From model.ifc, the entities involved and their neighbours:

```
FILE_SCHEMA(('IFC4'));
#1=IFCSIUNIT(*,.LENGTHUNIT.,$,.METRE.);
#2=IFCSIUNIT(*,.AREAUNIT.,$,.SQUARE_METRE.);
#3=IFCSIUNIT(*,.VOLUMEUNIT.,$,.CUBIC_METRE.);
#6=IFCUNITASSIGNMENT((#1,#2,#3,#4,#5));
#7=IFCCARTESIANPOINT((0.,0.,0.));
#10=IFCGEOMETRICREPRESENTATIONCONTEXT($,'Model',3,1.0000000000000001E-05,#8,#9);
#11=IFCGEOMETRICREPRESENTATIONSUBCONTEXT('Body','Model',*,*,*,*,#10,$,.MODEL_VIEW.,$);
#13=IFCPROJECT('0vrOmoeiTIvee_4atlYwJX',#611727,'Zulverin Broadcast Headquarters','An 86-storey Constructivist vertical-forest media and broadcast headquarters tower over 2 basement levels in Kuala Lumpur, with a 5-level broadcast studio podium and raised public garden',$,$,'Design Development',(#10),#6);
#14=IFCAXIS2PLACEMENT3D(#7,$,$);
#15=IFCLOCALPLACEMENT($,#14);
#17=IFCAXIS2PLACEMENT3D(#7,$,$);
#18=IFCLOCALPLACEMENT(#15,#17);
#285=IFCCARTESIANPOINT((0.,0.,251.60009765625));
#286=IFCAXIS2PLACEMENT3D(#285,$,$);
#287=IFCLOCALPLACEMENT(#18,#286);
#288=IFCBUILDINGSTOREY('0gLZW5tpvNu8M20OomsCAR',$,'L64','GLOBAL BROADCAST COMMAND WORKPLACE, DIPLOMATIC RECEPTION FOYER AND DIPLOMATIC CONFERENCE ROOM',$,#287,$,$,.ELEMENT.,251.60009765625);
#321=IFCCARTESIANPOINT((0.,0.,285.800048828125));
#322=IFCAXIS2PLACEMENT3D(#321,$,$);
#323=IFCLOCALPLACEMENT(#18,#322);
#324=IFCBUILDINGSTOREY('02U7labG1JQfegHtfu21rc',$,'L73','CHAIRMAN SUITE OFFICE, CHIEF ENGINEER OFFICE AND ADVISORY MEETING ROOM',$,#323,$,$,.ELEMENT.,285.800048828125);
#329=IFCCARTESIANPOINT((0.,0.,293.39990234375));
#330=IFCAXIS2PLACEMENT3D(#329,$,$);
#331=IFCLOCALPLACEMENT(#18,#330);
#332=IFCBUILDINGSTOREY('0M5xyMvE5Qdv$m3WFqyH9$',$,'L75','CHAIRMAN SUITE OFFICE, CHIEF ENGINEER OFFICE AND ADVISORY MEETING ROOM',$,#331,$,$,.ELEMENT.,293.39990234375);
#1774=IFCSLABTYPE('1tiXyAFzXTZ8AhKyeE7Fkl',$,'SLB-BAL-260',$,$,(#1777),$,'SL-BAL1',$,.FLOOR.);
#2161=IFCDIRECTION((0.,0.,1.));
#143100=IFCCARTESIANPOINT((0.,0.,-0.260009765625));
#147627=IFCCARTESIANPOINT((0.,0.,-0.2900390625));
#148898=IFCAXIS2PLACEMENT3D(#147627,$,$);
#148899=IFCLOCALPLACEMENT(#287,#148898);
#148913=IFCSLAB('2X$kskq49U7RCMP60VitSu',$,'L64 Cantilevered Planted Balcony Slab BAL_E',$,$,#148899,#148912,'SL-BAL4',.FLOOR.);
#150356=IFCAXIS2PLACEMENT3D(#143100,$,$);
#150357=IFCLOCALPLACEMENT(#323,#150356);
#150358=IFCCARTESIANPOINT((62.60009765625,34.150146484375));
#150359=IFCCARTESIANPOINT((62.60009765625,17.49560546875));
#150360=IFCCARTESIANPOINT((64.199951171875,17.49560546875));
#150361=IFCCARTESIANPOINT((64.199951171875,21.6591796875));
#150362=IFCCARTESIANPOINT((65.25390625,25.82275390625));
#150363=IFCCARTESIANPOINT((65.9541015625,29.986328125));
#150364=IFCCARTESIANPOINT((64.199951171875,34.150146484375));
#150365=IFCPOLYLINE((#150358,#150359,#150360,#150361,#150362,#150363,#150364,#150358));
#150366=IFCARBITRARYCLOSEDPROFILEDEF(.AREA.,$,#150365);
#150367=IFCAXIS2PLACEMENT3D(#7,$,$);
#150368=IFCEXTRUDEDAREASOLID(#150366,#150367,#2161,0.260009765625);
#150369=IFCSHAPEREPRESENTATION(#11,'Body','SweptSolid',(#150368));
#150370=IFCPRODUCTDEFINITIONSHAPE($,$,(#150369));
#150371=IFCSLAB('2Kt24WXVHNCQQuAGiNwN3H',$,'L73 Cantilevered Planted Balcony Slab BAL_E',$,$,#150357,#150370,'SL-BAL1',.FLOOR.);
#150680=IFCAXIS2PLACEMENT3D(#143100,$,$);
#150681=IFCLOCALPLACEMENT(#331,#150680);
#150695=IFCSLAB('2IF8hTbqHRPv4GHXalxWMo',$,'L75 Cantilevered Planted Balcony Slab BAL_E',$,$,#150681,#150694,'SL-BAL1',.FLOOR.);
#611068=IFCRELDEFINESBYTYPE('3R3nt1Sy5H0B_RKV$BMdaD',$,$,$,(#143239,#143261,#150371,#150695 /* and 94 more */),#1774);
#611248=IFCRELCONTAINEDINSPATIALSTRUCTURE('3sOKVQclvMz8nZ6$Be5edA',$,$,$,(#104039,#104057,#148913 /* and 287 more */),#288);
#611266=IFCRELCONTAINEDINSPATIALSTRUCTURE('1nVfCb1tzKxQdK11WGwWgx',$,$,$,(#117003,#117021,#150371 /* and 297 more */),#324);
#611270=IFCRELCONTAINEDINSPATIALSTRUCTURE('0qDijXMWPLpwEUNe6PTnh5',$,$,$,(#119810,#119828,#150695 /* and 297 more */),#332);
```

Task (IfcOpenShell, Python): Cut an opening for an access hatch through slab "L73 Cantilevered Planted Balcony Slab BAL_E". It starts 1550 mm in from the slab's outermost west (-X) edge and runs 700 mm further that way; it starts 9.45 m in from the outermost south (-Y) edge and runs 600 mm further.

```python
import numpy as np
import ifcopenshell
import ifcopenshell.api.feature
import ifcopenshell.api.geometry
import ifcopenshell.api.root
import ifcopenshell.geom
import ifcopenshell.util.placement
import ifcopenshell.util.representation
import ifcopenshell.util.shape
import ifcopenshell.util.unit

model = ifcopenshell.open("model.ifc")
unit_scale = ifcopenshell.util.unit.calculate_unit_scale(model)
settings = ifcopenshell.geom.settings()


def volume(element):
    """Net volume in cubic metres, openings subtracted."""
    shape = ifcopenshell.geom.create_shape(settings, element)
    return ifcopenshell.util.shape.get_volume(shape.geometry)


slab = model.by_guid("2Kt24WXVHNCQQuAGiNwN3H")
before = volume(slab)

# Extent in the slab's own axes, in metres. The edges named are its -X and -Y sides.
slab_shape = ifcopenshell.geom.create_shape(settings, slab)
vertices = ifcopenshell.util.shape.get_vertices(slab_shape.geometry)
x_min, y_min, bottom = vertices.min(axis=0)
top = vertices[:, 2].max()

opening = ifcopenshell.api.root.create_entity(model, ifc_class="IfcOpeningElement", name="Access hatch opening", predefined_type="OPENING")
context = ifcopenshell.util.representation.get_context(model, "Model", "Body", "MODEL_VIEW")
width, depth = 0.7, 0.6
outline = [(0.0, 0.0), (width, 0.0), (width, depth), (0.0, depth), (0.0, 0.0)]
# Overshoot both faces by 50 mm so the cut is clean.
shape = ifcopenshell.api.geometry.add_slab_representation(
    model, context=context, depth=top - bottom + 0.1, polyline=outline
)
ifcopenshell.api.geometry.assign_representation(model, product=opening, representation=shape)

matrix = ifcopenshell.util.placement.get_local_placement(slab.ObjectPlacement)
matrix[:, 3] = matrix @ np.append(np.array([x_min + 1.55, y_min + 9.45, bottom - 0.05]) / unit_scale, 1.0)
ifcopenshell.api.geometry.edit_object_placement(model, product=opening, matrix=matrix, is_si=False)
ifcopenshell.api.feature.add_feature(model, feature=opening, element=slab)

after = volume(slab)

print(f"slab volume {before:.3f} -> {after:.3f} m3")

model.write("model_edited.ifc")
```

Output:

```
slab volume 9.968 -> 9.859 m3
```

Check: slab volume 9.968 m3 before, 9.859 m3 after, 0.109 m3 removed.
